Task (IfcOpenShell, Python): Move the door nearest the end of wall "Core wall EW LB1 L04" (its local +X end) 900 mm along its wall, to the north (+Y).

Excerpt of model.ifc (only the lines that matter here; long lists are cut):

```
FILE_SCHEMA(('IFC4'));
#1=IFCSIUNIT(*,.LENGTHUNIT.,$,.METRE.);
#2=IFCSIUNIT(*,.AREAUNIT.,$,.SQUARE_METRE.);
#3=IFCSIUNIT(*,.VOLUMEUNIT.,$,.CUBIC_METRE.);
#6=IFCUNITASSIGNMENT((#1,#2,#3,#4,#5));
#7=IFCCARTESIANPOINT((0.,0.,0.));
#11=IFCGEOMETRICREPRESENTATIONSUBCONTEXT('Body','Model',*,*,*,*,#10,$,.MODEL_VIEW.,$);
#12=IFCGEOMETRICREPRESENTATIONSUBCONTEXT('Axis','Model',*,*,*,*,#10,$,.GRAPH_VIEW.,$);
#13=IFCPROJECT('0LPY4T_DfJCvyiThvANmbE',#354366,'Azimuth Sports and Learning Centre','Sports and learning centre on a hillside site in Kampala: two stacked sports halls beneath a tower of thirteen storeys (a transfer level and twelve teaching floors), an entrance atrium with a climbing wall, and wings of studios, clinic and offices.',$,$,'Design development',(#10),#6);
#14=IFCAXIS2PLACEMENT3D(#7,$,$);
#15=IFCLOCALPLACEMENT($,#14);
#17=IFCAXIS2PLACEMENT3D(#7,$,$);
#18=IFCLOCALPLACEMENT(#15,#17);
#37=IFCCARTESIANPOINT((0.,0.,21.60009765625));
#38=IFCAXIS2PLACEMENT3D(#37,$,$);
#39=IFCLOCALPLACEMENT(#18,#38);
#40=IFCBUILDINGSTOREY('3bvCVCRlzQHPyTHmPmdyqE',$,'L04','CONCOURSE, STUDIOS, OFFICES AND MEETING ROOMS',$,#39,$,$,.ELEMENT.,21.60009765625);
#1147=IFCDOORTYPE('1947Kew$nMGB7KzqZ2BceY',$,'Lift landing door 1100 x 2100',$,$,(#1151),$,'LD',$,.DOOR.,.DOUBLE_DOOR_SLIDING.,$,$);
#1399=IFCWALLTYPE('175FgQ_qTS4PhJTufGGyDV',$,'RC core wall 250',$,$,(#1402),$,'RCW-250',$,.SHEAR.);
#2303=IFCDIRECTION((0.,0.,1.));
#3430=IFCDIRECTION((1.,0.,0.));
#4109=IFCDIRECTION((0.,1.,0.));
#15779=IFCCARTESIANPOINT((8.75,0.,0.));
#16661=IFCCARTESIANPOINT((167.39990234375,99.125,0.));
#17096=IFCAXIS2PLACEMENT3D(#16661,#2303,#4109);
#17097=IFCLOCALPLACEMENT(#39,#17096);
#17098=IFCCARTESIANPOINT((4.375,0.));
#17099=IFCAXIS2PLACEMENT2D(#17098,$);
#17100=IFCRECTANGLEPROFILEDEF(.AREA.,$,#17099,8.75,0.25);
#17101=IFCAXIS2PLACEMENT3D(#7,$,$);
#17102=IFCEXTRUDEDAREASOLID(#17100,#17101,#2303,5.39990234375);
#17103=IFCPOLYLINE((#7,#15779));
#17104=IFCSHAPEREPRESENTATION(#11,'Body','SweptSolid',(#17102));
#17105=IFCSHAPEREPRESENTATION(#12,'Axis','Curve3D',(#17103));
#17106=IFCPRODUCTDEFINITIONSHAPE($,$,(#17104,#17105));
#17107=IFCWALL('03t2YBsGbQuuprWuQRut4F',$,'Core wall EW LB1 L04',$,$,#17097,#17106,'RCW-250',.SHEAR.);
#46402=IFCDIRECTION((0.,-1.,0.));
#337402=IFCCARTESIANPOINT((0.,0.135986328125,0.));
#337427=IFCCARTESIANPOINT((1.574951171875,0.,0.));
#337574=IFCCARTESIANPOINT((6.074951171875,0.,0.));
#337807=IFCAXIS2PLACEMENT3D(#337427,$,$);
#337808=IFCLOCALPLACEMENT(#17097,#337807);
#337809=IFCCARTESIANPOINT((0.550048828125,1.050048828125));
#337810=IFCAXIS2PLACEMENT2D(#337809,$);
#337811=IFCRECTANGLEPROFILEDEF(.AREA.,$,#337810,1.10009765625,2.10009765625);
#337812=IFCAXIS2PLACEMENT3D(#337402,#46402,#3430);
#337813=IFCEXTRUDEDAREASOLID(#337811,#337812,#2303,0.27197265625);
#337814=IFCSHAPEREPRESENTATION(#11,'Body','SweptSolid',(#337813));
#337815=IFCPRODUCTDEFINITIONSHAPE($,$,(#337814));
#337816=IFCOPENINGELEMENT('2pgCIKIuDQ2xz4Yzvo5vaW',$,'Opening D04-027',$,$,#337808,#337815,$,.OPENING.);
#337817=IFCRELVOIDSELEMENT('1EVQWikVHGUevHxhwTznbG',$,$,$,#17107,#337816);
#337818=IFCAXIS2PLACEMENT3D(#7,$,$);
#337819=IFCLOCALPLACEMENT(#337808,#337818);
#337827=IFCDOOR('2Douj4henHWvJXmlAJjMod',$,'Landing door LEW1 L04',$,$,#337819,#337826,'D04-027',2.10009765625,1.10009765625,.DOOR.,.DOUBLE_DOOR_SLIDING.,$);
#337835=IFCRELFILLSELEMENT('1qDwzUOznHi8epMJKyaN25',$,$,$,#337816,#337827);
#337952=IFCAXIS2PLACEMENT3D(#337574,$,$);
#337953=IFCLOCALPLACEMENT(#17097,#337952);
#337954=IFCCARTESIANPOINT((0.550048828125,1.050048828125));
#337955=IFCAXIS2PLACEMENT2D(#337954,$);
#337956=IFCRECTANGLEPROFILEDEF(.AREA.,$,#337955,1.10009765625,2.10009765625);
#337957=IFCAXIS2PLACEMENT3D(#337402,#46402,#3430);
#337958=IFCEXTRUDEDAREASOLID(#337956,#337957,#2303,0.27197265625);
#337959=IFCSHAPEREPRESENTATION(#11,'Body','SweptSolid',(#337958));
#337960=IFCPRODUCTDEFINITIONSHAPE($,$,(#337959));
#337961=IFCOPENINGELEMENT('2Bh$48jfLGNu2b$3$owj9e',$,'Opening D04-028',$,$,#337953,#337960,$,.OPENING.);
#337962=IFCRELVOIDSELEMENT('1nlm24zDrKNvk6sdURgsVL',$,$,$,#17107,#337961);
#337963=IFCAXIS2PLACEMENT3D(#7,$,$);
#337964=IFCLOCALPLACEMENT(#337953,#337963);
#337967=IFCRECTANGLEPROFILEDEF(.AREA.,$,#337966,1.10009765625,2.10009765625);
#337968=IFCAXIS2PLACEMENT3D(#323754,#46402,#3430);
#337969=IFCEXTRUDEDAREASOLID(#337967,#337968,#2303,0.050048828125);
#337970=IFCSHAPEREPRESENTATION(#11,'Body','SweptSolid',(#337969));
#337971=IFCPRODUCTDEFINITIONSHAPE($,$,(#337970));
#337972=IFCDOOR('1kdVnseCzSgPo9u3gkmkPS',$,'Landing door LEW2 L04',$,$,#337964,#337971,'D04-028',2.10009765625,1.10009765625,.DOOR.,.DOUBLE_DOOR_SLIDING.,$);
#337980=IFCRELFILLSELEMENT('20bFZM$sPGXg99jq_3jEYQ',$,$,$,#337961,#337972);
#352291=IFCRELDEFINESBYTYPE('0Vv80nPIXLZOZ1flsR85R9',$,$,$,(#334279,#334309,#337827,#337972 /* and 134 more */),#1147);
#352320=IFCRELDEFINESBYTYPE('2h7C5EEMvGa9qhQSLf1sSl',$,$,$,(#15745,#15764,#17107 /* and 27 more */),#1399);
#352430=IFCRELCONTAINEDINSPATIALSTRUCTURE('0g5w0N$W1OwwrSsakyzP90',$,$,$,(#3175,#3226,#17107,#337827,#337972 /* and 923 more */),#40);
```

```python
import ifcopenshell
import ifcopenshell.api.geometry
import ifcopenshell.util.placement
import ifcopenshell.util.unit

model = ifcopenshell.open("model.ifc")
unit_scale = ifcopenshell.util.unit.calculate_unit_scale(model)

door = model.by_guid("1kdVnseCzSgPo9u3gkmkPS")
opening = door.FillsVoids[0].RelatingOpeningElement
wall = opening.VoidsElements[0].RelatingBuildingElement

wall_matrix = ifcopenshell.util.placement.get_local_placement(wall.ObjectPlacement)
shift = wall_matrix[:3, 0] * 0.9 / unit_scale
before = ifcopenshell.util.placement.get_local_placement(door.ObjectPlacement)[:3, 3].copy()

# The door is placed relative to its opening, so it follows when the opening moves.
matrix = ifcopenshell.util.placement.get_local_placement(opening.ObjectPlacement)
matrix[:3, 3] += shift
ifcopenshell.api.geometry.edit_object_placement(
    model, product=opening, matrix=matrix, is_si=False, should_transform_children=True
)

after = ifcopenshell.util.placement.get_local_placement(door.ObjectPlacement)[:3, 3]
print("door moved by", (after - before).round(3) + 0.0)

model.write("model_rev.ifc")
```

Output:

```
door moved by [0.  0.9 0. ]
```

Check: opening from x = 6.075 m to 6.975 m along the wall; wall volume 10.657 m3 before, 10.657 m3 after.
